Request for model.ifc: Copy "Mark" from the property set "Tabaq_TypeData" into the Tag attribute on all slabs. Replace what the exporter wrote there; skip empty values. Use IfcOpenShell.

First a look at what the model holds.

```python
import ifcopenshell
import ifcopenshell.util.element

model = ifcopenshell.open("model.ifc")
print(model.schema)
slabs = model.by_type("IfcSlab")
print(len(slabs), "slabs")
for e in slabs[:8]:
    source = ifcopenshell.util.element.get_pset(e, "Tabaq_TypeData", "Mark")
    target = e.Tag
    print(e.id(), repr(source), repr(target), sep=" | ")
```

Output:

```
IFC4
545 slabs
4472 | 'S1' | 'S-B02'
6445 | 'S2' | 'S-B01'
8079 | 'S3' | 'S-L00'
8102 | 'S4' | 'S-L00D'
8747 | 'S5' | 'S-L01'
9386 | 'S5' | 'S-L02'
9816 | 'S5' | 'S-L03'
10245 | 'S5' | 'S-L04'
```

```python
import ifcopenshell
import ifcopenshell.util.element

model = ifcopenshell.open("model.ifc")

count = 0
for e in model.by_type("IfcSlab"):
    value = ifcopenshell.util.element.get_pset(e, "Tabaq_TypeData", "Mark")
    current = e.Tag
    if not value or not value.strip() or current == value:
        continue
    e.Tag = value
    count += 1

print(count, "slabs updated")

model.write("model_edited.ifc")
```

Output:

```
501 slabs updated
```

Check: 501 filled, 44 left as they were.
